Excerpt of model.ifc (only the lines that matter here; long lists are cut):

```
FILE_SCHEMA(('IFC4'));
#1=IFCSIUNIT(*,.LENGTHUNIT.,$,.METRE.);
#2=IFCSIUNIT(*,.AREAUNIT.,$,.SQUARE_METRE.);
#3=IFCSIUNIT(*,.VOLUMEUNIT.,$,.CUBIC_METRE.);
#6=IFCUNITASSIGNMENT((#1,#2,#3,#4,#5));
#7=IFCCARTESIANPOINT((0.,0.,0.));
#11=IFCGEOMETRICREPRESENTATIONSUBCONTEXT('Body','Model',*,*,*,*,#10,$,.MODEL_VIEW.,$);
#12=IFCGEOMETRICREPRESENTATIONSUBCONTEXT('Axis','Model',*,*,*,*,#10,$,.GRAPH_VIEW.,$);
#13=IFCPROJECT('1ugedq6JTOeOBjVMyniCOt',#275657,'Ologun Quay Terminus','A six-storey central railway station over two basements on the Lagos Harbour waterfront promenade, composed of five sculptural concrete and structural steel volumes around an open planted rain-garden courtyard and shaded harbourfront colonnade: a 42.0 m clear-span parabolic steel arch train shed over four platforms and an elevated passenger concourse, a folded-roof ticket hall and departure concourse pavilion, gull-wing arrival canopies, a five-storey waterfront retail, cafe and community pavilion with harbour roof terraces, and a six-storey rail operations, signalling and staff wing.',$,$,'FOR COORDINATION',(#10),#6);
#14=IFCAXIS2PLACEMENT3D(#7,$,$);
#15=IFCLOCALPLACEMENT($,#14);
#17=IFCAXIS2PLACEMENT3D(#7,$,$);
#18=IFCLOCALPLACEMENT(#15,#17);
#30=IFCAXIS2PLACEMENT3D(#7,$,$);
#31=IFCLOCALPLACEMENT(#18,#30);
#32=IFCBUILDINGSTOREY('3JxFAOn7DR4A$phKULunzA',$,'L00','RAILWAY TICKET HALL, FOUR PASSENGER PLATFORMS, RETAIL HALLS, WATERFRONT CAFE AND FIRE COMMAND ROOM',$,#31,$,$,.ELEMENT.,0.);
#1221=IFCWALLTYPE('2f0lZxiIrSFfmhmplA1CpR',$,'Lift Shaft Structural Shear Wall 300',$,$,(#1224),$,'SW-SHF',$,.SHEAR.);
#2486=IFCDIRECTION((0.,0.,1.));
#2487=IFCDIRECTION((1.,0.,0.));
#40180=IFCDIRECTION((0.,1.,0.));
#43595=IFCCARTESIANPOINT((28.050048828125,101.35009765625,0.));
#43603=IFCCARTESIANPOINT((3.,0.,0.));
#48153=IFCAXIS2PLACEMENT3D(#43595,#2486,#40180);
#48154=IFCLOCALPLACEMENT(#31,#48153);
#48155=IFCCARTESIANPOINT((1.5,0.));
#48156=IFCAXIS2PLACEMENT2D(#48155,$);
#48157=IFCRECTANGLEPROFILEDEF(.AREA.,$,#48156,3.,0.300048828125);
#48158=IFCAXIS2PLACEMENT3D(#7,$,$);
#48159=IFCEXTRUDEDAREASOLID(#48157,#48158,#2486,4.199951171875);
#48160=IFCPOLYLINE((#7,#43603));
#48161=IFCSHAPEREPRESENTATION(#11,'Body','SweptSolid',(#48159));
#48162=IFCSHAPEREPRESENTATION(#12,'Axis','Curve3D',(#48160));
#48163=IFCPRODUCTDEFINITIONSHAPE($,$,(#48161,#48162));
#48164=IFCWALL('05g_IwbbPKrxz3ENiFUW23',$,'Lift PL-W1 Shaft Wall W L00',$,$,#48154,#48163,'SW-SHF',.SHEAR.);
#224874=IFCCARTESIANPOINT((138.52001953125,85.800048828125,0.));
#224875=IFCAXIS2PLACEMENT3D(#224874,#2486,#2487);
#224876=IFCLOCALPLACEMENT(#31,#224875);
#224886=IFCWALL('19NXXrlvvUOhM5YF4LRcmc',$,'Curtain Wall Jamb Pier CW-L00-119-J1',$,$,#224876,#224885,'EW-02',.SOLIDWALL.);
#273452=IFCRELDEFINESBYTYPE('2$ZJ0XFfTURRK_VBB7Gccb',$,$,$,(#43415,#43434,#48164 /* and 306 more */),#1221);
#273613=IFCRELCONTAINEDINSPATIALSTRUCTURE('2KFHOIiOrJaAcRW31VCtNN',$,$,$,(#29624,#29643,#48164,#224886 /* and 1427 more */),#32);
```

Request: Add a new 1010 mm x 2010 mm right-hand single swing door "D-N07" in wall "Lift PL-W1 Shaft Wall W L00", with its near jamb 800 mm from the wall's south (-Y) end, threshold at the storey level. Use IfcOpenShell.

```python
import numpy as np
import ifcopenshell
import ifcopenshell.api.feature
import ifcopenshell.api.geometry
import ifcopenshell.api.root
import ifcopenshell.api.spatial
import ifcopenshell.geom
import ifcopenshell.util.element
import ifcopenshell.util.placement
import ifcopenshell.util.representation
import ifcopenshell.util.shape
import ifcopenshell.util.unit

model = ifcopenshell.open("model.ifc")
unit_scale = ifcopenshell.util.unit.calculate_unit_scale(model)
settings = ifcopenshell.geom.settings()


def volume(element):
    """Net volume in cubic metres, openings subtracted."""
    shape = ifcopenshell.geom.create_shape(settings, element)
    return ifcopenshell.util.shape.get_volume(shape.geometry)


wall = model.by_guid("05g_IwbbPKrxz3ENiFUW23")
storey = ifcopenshell.util.element.get_container(wall, ifc_class="IfcBuildingStorey")
context = ifcopenshell.util.representation.get_context(model, "Model", "Body", "MODEL_VIEW")
before = volume(wall)

width, height, from_end, sill = 1.01, 2.01, 0.8, 0.0  # metres

# The wall runs along its own X axis, and the end named is its -X end.
wall_shape = ifcopenshell.geom.create_shape(settings, wall)
x, y, z = ifcopenshell.util.shape.get_vertices(wall_shape.geometry).T
start = x.min() + from_end
face, thickness = float(y.min()), float(y.max() - y.min())
wall_matrix = ifcopenshell.util.placement.get_local_placement(wall.ObjectPlacement)
level = ifcopenshell.util.placement.get_local_placement(storey.ObjectPlacement)[2, 3]


def in_wall(x, y):
    """Placement at x, y metres in the wall's axes, at sill height."""
    matrix = wall_matrix.copy()
    matrix[:, 3] = wall_matrix @ np.array([x / unit_scale, y / unit_scale, 0.0, 1.0])
    matrix[2, 3] = level + sill / unit_scale
    return matrix


# Opening: a box that overshoots both wall faces by 50 mm.
opening = ifcopenshell.api.root.create_entity(model, ifc_class="IfcOpeningElement", predefined_type="OPENING")
box = ifcopenshell.api.geometry.add_wall_representation(
    model, context=context, length=width, height=height, thickness=thickness + 0.1
)
ifcopenshell.api.geometry.assign_representation(model, product=opening, representation=box)
ifcopenshell.api.geometry.edit_object_placement(model, product=opening, matrix=in_wall(start, face - 0.05), is_si=False)
ifcopenshell.api.feature.add_feature(model, feature=opening, element=wall)

door = ifcopenshell.api.root.create_entity(model, ifc_class="IfcDoor", name="D-N07", predefined_type="DOOR")
door.OverallWidth, door.OverallHeight = width / unit_scale, height / unit_scale
door.OperationType = "SINGLE_SWING_RIGHT"
body = ifcopenshell.api.geometry.add_door_representation(
    model,
    context=context,
    overall_width=door.OverallWidth,
    overall_height=door.OverallHeight,
    operation_type="SINGLE_SWING_RIGHT",
    lining_properties={"LiningDepth": thickness / unit_scale, "ThresholdDepth": thickness / unit_scale},
)
ifcopenshell.api.geometry.assign_representation(model, product=door, representation=body)
ifcopenshell.api.spatial.assign_container(model, products=[door], relating_structure=storey)
ifcopenshell.api.feature.add_filling(model, opening=opening, element=door)

# The lining spans the wall, so the door starts at the wall face.
ifcopenshell.api.geometry.edit_object_placement(model, product=door, matrix=in_wall(start, face), is_si=False)

after = volume(wall)

print(f"wall volume {before:.3f} -> {after:.3f} m3")

model.write("model_edited.ifc")
```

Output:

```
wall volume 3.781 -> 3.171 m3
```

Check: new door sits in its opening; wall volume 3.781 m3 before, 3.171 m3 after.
